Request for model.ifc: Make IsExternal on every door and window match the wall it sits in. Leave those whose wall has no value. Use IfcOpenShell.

First a look at what the model holds.

```python
import ifcopenshell
import ifcopenshell.util.element

model = ifcopenshell.open("model.ifc")
print(model.schema)
seen = {}
for e in model.by_type("IfcDoor") + model.by_type("IfcWindow"):
    if not e.FillsVoids:
        continue
    host = e.FillsVoids[0].RelatingOpeningElement.VoidsElements[0].RelatingBuildingElement
    own = ifcopenshell.util.element.get_pset(e, f"Pset_{e.is_a()[3:].removesuffix('StandardCase')}Common", "IsExternal")
    wall = ifcopenshell.util.element.get_pset(host, "Pset_WallCommon", "IsExternal")
    seen[e.is_a(), own, wall] = seen.get((e.is_a(), own, wall), 0) + 1
for (cls, own, wall), count in sorted(seen.items(), key=str):
    print(count, cls, "IsExternal:", own, "| host wall:", wall)
```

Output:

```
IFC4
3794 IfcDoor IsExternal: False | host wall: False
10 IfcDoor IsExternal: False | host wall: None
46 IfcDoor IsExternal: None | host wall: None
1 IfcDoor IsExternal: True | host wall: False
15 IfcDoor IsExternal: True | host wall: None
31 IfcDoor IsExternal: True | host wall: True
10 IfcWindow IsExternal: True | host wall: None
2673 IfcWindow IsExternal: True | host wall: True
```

```python
import ifcopenshell
import ifcopenshell.api.pset
import ifcopenshell.util.element

model = ifcopenshell.open("model.ifc")

count = 0
for ifc_class, pset_name in (("IfcDoor", "Pset_DoorCommon"), ("IfcWindow", "Pset_WindowCommon")):
    for e in model.by_type(ifc_class):
        if not e.FillsVoids:
            continue
        host = e.FillsVoids[0].RelatingOpeningElement.VoidsElements[0].RelatingBuildingElement
        external = ifcopenshell.util.element.get_pset(host, "Pset_WallCommon", "IsExternal")
        if external is None or ifcopenshell.util.element.get_pset(e, pset_name, "IsExternal") == external:
            continue
        pset = ifcopenshell.api.pset.add_pset(model, product=e, name=pset_name)
        ifcopenshell.api.pset.edit_pset(model, pset=pset, properties={"IsExternal": external})
        count += 1

print(count, "updated")

model.write("model_updated.ifc")
```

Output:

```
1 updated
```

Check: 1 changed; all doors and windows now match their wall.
